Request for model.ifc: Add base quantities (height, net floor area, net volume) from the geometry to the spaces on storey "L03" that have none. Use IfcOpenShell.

First a look at what the model holds.

```python
import ifcopenshell
import ifcopenshell.util.element
import ifcopenshell.util.unit

model = ifcopenshell.open("model.ifc")
print(model.schema)
for unit_type in ("LENGTHUNIT", "AREAUNIT", "VOLUMEUNIT"):
    print(unit_type, ifcopenshell.util.unit.calculate_unit_scale(model, unit_type))
storey = next(s for s in model.by_type("IfcBuildingStorey") if s.Name == "L03")
spaces = [e for e in ifcopenshell.util.element.get_decomposition(storey) if e.is_a("IfcSpace")]
for e in sorted(spaces, key=lambda e: e.id()):
    print(e.id(), e.is_a(), e.Name, list(ifcopenshell.util.element.get_psets(e, qtos_only=True)), sep=" | ")
```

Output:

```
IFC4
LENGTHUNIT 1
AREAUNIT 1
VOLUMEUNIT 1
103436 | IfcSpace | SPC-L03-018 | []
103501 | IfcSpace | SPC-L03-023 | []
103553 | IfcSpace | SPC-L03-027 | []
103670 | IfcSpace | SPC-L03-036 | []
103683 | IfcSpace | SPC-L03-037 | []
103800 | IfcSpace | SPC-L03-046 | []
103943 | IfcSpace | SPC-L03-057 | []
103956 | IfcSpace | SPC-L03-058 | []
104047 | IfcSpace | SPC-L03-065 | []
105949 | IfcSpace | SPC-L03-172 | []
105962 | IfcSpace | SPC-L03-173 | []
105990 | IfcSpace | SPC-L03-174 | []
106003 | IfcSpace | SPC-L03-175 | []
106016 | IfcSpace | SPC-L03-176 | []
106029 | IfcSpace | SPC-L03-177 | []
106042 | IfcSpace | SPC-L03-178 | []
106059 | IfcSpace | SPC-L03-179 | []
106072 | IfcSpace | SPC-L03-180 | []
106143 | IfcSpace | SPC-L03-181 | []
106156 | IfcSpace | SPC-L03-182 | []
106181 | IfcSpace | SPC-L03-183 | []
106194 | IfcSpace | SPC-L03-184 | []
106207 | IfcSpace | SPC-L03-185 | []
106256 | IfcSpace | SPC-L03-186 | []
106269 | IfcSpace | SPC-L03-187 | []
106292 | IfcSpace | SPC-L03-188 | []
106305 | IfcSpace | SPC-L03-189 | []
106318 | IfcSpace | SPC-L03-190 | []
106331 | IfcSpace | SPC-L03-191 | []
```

```python
import ifcopenshell
import ifcopenshell.api.pset
import ifcopenshell.geom
import ifcopenshell.util.element
import ifcopenshell.util.shape
import ifcopenshell.util.unit

model = ifcopenshell.open("model.ifc")
unit_scale = ifcopenshell.util.unit.calculate_unit_scale(model)
area_scale = ifcopenshell.util.unit.calculate_unit_scale(model, "AREAUNIT")
volume_scale = ifcopenshell.util.unit.calculate_unit_scale(model, "VOLUMEUNIT")
settings = ifcopenshell.geom.settings()

storey = next(s for s in model.by_type("IfcBuildingStorey") if s.Name == "L03")
spaces = [e for e in ifcopenshell.util.element.get_decomposition(storey) if e.is_a("IfcSpace")]

for e in sorted(spaces, key=lambda e: e.id()):
    if ifcopenshell.util.element.get_psets(e, qtos_only=True, should_inherit=False):
        continue
    # Geometry comes back in metres, in the element's own axes.
    shape = ifcopenshell.geom.create_shape(settings, e)
    values = {
        "Height": ifcopenshell.util.shape.get_z(shape.geometry) / unit_scale,
        "NetFloorArea": ifcopenshell.util.shape.get_footprint_area(shape.geometry) / area_scale,
        "NetVolume": ifcopenshell.util.shape.get_volume(shape.geometry) / volume_scale,
    }
    qto = ifcopenshell.api.pset.add_qto(model, product=e, name="Qto_SpaceBaseQuantities")
    ifcopenshell.api.pset.edit_qto(model, qto=qto, properties=values)
    print(e.id(), {k: round(v, 3) for k, v in values.items()})

model.write("model_updated.ifc")
```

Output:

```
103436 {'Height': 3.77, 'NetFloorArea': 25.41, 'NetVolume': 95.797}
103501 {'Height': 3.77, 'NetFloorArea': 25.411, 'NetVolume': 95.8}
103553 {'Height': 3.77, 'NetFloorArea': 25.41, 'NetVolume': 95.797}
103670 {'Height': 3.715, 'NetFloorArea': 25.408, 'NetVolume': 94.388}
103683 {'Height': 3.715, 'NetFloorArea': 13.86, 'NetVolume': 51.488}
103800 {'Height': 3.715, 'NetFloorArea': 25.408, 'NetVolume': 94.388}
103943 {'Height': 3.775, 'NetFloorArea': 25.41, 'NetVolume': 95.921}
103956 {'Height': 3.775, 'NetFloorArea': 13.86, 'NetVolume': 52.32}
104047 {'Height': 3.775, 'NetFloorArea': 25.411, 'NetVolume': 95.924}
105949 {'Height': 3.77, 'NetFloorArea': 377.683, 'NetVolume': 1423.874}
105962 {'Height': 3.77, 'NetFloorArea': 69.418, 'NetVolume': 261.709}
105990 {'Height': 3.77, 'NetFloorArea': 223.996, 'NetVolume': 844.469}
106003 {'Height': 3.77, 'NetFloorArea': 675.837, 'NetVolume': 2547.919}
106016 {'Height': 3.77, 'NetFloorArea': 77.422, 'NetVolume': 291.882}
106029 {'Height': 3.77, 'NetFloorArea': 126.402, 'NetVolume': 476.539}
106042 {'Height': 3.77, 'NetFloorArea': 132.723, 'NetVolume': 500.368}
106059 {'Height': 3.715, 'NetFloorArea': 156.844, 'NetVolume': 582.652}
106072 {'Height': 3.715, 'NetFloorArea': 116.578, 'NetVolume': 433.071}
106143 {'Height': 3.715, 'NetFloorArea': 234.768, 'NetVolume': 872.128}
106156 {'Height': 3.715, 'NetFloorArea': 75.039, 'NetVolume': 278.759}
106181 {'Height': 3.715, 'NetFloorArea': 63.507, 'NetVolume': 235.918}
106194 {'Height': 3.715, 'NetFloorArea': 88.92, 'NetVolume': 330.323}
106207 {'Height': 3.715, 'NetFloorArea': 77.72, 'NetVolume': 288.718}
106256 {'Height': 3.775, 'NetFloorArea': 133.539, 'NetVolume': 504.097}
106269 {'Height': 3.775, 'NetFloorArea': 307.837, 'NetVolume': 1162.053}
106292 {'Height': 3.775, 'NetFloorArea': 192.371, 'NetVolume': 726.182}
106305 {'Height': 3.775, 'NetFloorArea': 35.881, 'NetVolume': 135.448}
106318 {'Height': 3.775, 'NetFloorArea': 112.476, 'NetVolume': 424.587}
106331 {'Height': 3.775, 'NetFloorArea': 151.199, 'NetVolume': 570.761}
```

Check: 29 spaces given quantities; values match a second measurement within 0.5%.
